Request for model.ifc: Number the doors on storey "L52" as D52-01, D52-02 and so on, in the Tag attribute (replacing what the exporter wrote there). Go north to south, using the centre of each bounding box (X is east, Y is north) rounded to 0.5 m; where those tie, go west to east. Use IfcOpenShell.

First a look at what the model holds.

```python
import ifcopenshell
import ifcopenshell.util.element
import ifcopenshell.util.placement

model = ifcopenshell.open("model.ifc")
print(model.schema)
storey = next(s for s in model.by_type("IfcBuildingStorey") if s.Name == "L52")
doors = [e for e in ifcopenshell.util.element.get_decomposition(storey) if e.is_a("IfcDoor")]
for e in sorted(doors, key=lambda e: e.id()):
    origin = ifcopenshell.util.placement.get_local_placement(e.ObjectPlacement)[:3, 3]
    print(e.id(), e.Tag, e.Name, origin.round(2) + 0.0, sep=" | ")
```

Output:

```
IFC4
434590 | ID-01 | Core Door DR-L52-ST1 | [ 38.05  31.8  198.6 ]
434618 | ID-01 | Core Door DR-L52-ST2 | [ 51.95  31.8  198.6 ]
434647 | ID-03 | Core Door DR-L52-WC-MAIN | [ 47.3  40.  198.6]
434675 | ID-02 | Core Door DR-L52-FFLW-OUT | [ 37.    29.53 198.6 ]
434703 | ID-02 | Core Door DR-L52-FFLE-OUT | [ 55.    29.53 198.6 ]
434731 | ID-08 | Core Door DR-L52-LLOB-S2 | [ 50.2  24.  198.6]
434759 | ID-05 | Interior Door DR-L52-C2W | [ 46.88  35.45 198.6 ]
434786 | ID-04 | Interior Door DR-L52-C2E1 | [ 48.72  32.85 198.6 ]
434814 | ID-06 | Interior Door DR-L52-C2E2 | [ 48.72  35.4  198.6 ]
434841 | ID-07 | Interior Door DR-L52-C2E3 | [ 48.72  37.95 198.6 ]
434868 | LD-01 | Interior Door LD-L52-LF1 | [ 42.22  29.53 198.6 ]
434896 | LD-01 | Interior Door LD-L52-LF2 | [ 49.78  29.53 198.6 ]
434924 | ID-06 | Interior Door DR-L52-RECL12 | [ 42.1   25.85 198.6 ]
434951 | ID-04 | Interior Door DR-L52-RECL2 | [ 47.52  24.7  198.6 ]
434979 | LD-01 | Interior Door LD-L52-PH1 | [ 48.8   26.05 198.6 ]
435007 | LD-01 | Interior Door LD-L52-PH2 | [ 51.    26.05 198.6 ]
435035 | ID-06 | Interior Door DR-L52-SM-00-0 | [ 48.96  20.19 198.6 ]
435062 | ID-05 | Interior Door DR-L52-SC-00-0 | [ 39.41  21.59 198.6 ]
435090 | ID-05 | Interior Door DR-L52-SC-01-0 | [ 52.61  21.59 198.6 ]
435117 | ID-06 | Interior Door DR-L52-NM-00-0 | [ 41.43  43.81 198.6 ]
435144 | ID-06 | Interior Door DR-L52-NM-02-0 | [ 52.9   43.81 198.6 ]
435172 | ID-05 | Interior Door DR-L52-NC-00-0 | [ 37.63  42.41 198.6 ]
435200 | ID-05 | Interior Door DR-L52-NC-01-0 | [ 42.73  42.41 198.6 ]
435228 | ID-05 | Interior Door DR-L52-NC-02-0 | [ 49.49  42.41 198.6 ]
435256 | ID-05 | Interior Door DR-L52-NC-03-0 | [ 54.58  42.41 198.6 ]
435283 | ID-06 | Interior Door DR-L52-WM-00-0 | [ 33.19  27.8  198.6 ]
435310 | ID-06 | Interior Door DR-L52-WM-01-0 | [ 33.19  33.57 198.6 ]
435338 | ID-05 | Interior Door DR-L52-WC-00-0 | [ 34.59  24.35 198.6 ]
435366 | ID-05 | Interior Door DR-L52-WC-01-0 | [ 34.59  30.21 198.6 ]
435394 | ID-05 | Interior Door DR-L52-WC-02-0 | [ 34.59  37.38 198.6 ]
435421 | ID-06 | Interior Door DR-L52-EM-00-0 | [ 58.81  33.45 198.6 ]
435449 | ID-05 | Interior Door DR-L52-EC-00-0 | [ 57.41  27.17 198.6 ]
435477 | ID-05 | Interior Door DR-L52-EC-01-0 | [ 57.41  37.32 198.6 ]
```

```python
import ifcopenshell
import ifcopenshell.geom
import ifcopenshell.util.element
import ifcopenshell.util.shape

model = ifcopenshell.open("model.ifc")
settings = ifcopenshell.geom.settings()
settings.set("use-world-coords", True)


def centre(element):
    shape = ifcopenshell.geom.create_shape(settings, element)
    return ifcopenshell.util.shape.get_bbox_centroid(shape.geometry)


storey = next(s for s in model.by_type("IfcBuildingStorey") if s.Name == "L52")
doors = [e for e in ifcopenshell.util.element.get_decomposition(storey) if e.is_a("IfcDoor")]

# Insertion points can sit at a corner or the storey origin, so sort by the geometry (in metres).
centres = {e: centre(e) for e in doors}
doors.sort(key=lambda e: (-round(centres[e][1] / 0.5), centres[e][0]))

for i, e in enumerate(doors, start=1):
    number = f"D52-{i:02d}"
    e.Tag = number
    print(e.id(), number)

model.write("model-out.ifc")
```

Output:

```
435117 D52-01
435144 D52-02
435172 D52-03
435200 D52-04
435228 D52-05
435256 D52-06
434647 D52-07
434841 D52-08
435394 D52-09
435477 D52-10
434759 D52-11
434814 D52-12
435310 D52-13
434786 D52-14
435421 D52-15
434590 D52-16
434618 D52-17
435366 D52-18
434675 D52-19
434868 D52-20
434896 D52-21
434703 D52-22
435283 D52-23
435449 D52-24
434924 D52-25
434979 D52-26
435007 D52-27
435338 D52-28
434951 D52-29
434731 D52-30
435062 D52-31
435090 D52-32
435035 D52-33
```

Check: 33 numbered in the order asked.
